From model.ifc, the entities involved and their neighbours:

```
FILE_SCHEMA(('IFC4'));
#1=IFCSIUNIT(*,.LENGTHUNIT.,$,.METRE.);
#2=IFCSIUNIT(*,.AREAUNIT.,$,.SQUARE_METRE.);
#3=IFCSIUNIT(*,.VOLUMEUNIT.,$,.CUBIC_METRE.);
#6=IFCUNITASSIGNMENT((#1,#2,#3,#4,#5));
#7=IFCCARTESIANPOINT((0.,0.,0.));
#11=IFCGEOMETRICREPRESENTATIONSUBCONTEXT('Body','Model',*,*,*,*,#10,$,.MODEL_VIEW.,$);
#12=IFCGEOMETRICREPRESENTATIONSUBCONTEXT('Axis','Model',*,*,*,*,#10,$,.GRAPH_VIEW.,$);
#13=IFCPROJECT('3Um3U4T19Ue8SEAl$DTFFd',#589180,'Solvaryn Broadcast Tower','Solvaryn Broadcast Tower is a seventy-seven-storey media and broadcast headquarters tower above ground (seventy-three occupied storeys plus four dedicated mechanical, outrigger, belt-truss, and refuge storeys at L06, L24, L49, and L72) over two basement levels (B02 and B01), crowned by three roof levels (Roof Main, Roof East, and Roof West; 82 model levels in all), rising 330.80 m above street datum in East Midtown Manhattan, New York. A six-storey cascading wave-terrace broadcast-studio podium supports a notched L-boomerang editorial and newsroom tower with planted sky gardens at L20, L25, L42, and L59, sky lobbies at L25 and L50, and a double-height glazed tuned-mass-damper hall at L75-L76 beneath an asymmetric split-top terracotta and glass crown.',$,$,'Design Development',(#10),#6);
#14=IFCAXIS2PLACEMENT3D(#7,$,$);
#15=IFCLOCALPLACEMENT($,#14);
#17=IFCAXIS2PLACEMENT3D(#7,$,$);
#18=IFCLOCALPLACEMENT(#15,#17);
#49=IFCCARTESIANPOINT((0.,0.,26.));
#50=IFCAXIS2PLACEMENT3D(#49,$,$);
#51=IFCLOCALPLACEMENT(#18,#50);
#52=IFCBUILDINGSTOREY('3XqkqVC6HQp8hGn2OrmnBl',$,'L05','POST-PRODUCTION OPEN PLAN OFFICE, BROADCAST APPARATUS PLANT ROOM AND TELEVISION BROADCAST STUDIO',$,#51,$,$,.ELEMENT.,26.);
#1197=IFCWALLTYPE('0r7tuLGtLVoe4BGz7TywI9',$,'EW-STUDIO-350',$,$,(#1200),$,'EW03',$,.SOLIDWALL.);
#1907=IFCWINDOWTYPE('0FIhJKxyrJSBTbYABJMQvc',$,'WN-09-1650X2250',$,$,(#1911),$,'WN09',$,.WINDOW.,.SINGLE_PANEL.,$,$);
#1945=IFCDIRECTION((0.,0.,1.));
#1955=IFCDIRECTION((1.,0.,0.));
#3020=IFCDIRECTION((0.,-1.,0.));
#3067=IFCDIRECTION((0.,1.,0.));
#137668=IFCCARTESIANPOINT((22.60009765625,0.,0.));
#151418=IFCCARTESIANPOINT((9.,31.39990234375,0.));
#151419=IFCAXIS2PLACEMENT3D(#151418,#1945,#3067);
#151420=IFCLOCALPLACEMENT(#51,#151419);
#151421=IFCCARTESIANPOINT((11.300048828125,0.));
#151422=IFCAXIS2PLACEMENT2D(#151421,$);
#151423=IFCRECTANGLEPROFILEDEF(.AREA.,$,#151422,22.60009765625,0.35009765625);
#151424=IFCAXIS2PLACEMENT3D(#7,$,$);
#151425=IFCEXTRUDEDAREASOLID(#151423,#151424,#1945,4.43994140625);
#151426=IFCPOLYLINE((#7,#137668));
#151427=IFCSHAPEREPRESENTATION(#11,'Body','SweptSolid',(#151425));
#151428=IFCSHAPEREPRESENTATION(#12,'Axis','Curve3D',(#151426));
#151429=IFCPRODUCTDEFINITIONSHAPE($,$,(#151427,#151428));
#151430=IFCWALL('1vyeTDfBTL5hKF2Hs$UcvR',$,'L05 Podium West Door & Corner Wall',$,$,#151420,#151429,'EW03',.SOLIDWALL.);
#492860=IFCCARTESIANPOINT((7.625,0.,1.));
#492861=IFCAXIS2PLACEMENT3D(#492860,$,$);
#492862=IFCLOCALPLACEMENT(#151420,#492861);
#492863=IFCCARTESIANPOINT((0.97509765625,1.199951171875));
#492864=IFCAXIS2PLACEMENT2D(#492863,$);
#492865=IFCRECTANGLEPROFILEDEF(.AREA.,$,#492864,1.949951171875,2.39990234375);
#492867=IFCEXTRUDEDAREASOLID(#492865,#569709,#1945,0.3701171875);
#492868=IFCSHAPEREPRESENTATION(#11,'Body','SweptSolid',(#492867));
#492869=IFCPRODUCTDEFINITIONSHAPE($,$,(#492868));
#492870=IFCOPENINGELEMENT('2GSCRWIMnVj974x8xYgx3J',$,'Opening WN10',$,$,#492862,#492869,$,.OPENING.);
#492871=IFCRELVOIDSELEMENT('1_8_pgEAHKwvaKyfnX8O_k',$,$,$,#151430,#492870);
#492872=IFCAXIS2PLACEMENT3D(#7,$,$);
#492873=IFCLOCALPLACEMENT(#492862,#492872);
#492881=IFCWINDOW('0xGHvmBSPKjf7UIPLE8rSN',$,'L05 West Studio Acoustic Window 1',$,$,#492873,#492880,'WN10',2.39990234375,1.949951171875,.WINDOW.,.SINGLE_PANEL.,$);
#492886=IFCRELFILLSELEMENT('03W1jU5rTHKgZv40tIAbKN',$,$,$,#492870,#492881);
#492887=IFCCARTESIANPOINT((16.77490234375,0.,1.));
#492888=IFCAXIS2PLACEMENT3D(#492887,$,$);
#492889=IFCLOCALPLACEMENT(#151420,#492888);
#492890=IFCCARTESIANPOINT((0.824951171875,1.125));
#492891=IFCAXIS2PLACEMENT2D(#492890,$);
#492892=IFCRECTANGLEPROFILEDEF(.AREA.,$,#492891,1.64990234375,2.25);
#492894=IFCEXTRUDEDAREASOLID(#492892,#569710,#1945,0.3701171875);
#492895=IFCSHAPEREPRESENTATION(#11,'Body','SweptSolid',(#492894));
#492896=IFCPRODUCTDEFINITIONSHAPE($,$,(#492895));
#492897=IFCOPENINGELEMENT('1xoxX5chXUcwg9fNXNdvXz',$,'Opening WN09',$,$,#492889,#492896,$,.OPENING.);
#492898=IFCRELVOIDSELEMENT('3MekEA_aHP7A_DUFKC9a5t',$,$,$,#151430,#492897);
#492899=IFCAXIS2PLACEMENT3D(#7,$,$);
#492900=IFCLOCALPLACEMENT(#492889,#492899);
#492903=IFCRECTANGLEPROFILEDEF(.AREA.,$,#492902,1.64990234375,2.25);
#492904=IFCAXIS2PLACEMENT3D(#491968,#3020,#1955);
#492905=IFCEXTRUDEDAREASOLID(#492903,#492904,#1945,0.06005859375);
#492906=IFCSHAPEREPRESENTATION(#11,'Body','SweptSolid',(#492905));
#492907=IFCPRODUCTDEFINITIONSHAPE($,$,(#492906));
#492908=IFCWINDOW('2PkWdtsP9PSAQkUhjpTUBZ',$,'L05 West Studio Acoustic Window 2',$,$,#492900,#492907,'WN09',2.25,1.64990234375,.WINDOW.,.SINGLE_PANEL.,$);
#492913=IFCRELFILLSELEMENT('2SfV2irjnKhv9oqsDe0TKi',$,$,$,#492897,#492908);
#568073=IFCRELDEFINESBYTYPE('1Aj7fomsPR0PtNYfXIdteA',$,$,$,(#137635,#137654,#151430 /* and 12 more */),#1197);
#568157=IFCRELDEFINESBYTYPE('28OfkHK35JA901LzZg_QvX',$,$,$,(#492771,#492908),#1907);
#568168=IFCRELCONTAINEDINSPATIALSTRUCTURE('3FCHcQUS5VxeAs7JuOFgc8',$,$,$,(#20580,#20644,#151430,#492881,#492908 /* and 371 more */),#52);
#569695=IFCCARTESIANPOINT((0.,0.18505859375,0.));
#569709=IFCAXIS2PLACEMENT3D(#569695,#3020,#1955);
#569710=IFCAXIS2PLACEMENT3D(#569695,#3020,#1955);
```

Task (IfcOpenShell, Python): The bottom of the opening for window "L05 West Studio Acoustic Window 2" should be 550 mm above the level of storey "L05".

```python
import numpy as np
import ifcopenshell
import ifcopenshell.api.geometry
import ifcopenshell.geom
import ifcopenshell.util.element
import ifcopenshell.util.placement
import ifcopenshell.util.shape
import ifcopenshell.util.unit

model = ifcopenshell.open("model.ifc")
unit_scale = ifcopenshell.util.unit.calculate_unit_scale(model)

window = model.by_guid("2PkWdtsP9PSAQkUhjpTUBZ")
opening = window.FillsVoids[0].RelatingOpeningElement
storey = ifcopenshell.util.element.get_container(window, ifc_class="IfcBuildingStorey")
level = ifcopenshell.util.placement.get_local_placement(storey.ObjectPlacement)[2, 3]

# The opening's origin need not be at the sill, so measure its lowest point.
shape = ifcopenshell.geom.create_shape(ifcopenshell.geom.settings(), opening)
bottom = ifcopenshell.util.shape.get_shape_bottom_elevation(shape, shape.geometry) / unit_scale
dz = level + 0.55 / unit_scale - bottom

shift = np.array([0.0, 0.0, dz])
# The window is placed relative to its opening, so it follows when the opening moves.
matrix = ifcopenshell.util.placement.get_local_placement(opening.ObjectPlacement)
matrix[:3, 3] += shift
ifcopenshell.api.geometry.edit_object_placement(
    model, product=opening, matrix=matrix, is_si=False, should_transform_children=True
)

print(f"moved by {dz * unit_scale:+.3f} m")

model.write("model_edited.ifc")
```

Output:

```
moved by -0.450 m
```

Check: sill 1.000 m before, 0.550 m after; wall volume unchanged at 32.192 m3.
